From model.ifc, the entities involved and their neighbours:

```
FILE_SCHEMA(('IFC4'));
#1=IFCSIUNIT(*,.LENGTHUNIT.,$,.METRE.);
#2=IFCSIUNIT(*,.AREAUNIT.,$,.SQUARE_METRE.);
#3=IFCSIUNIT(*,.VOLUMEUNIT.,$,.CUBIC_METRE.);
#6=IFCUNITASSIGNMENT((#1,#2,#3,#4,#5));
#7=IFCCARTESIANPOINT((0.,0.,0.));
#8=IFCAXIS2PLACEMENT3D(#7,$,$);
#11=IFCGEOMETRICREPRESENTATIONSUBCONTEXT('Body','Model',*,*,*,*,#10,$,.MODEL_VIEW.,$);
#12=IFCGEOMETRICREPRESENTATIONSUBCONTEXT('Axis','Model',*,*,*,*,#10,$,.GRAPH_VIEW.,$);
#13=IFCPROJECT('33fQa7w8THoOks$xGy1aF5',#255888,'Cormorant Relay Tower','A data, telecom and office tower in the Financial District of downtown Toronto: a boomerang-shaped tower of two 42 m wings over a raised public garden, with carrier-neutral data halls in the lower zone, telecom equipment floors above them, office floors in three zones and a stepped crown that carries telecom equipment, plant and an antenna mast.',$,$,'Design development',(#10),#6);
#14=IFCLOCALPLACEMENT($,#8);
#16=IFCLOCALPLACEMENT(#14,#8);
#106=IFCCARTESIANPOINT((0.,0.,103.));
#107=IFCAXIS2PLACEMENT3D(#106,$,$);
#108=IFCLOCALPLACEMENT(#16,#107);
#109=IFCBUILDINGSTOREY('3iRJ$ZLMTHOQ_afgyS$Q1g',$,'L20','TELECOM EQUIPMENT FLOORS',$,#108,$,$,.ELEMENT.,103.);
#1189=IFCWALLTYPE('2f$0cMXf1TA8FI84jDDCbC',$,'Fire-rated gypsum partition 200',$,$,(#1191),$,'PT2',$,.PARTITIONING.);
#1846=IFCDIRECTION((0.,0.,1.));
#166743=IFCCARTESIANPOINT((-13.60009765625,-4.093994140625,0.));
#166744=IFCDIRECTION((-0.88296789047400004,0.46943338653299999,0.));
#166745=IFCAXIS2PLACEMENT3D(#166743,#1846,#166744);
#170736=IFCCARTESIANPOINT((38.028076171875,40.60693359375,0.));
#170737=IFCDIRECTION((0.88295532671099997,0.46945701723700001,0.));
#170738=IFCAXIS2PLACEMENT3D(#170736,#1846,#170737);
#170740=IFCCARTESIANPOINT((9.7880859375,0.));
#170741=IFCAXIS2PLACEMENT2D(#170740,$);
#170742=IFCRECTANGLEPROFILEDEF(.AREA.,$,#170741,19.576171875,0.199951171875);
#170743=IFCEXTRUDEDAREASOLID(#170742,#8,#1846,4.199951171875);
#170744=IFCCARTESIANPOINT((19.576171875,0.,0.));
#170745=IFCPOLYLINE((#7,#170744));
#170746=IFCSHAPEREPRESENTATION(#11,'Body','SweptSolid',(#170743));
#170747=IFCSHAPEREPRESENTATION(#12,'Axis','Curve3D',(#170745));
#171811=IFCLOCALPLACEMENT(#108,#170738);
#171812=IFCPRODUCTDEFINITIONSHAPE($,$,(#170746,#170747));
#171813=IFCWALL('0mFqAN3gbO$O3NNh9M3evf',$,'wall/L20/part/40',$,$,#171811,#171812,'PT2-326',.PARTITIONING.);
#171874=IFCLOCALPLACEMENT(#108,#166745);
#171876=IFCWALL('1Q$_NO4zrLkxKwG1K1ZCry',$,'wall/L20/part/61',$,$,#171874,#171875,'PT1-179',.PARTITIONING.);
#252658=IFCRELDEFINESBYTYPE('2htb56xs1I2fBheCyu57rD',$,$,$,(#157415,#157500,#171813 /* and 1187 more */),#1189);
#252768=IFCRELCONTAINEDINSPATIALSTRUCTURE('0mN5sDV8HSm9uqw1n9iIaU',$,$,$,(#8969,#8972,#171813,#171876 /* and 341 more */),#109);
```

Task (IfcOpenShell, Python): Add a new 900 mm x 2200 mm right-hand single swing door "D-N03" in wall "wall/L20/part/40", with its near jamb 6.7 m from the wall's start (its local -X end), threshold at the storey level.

```python
import numpy as np
import ifcopenshell
import ifcopenshell.api.feature
import ifcopenshell.api.geometry
import ifcopenshell.api.root
import ifcopenshell.api.spatial
import ifcopenshell.geom
import ifcopenshell.util.element
import ifcopenshell.util.placement
import ifcopenshell.util.representation
import ifcopenshell.util.shape
import ifcopenshell.util.unit

model = ifcopenshell.open("model.ifc")
unit_scale = ifcopenshell.util.unit.calculate_unit_scale(model)
settings = ifcopenshell.geom.settings()


def volume(element):
    """Net volume in cubic metres, openings subtracted."""
    shape = ifcopenshell.geom.create_shape(settings, element)
    return ifcopenshell.util.shape.get_volume(shape.geometry)


wall = model.by_guid("0mFqAN3gbO$O3NNh9M3evf")
storey = ifcopenshell.util.element.get_container(wall, ifc_class="IfcBuildingStorey")
context = ifcopenshell.util.representation.get_context(model, "Model", "Body", "MODEL_VIEW")
before = volume(wall)

width, height, from_end, sill = 0.9, 2.2, 6.7, 0.0  # metres

# The wall runs along its own X axis, and the end named is its -X end.
wall_shape = ifcopenshell.geom.create_shape(settings, wall)
x, y, z = ifcopenshell.util.shape.get_vertices(wall_shape.geometry).T
start = x.min() + from_end
face, thickness = float(y.min()), float(y.max() - y.min())
wall_matrix = ifcopenshell.util.placement.get_local_placement(wall.ObjectPlacement)
level = ifcopenshell.util.placement.get_local_placement(storey.ObjectPlacement)[2, 3]


def in_wall(x, y):
    """Placement at x, y metres in the wall's axes, at sill height."""
    matrix = wall_matrix.copy()
    matrix[:, 3] = wall_matrix @ np.array([x / unit_scale, y / unit_scale, 0.0, 1.0])
    matrix[2, 3] = level + sill / unit_scale
    return matrix


# Opening: a box that overshoots both wall faces by 50 mm.
opening = ifcopenshell.api.root.create_entity(model, ifc_class="IfcOpeningElement", predefined_type="OPENING")
box = ifcopenshell.api.geometry.add_wall_representation(
    model, context=context, length=width, height=height, thickness=thickness + 0.1
)
ifcopenshell.api.geometry.assign_representation(model, product=opening, representation=box)
ifcopenshell.api.geometry.edit_object_placement(model, product=opening, matrix=in_wall(start, face - 0.05), is_si=False)
ifcopenshell.api.feature.add_feature(model, feature=opening, element=wall)

door = ifcopenshell.api.root.create_entity(model, ifc_class="IfcDoor", name="D-N03", predefined_type="DOOR")
door.OverallWidth, door.OverallHeight = width / unit_scale, height / unit_scale
door.OperationType = "SINGLE_SWING_RIGHT"
body = ifcopenshell.api.geometry.add_door_representation(
    model,
    context=context,
    overall_width=door.OverallWidth,
    overall_height=door.OverallHeight,
    operation_type="SINGLE_SWING_RIGHT",
    lining_properties={"LiningDepth": thickness / unit_scale, "ThresholdDepth": thickness / unit_scale},
)
ifcopenshell.api.geometry.assign_representation(model, product=door, representation=body)
ifcopenshell.api.spatial.assign_container(model, products=[door], relating_structure=storey)
ifcopenshell.api.feature.add_filling(model, opening=opening, element=door)

# The lining spans the wall, so the door starts at the wall face.
ifcopenshell.api.geometry.edit_object_placement(model, product=door, matrix=in_wall(start, face), is_si=False)

after = volume(wall)

print(f"wall volume {before:.3f} -> {after:.3f} m3")

model.write("model_rev.ifc")
```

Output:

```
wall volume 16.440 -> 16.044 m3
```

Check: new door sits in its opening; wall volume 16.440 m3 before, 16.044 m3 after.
